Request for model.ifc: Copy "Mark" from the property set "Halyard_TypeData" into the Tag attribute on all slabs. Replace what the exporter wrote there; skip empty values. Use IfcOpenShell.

First a look at what the model holds.

```python
import ifcopenshell
import ifcopenshell.util.element

model = ifcopenshell.open("model.ifc")
print(model.schema)
slabs = model.by_type("IfcSlab")
print(len(slabs), "slabs")
for e in slabs[:8]:
    source = ifcopenshell.util.element.get_pset(e, "Halyard_TypeData", "Mark")
    target = e.Tag
    print(e.id(), repr(source), repr(target), sep=" | ")
```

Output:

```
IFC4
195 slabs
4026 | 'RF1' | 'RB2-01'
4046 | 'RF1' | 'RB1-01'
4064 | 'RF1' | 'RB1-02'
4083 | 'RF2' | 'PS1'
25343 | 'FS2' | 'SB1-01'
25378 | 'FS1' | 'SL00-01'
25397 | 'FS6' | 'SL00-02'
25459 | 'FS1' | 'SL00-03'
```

```python
import ifcopenshell
import ifcopenshell.util.element

model = ifcopenshell.open("model.ifc")

count = 0
for e in model.by_type("IfcSlab"):
    value = ifcopenshell.util.element.get_pset(e, "Halyard_TypeData", "Mark")
    current = e.Tag
    if not value or not value.strip() or current == value:
        continue
    e.Tag = value
    count += 1

print(count, "slabs updated")

model.write("model-out.ifc")
```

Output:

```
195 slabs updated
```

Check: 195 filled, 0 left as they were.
